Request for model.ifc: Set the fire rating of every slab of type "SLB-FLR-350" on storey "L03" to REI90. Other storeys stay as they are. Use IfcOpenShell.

First a look at what the model holds.

```python
import ifcopenshell
import ifcopenshell.util.element

model = ifcopenshell.open("model.ifc")
print(model.schema)
storey = next(s for s in model.by_type("IfcBuildingStorey") if s.Name == "L03")
slabs = [e for e in ifcopenshell.util.element.get_decomposition(storey) if e.is_a("IfcSlab")]
seen = {}
for e in slabs:
    element_type = ifcopenshell.util.element.get_type(e)
    key = (element_type.Name if element_type != e and element_type else None, ifcopenshell.util.element.get_pset(e, "Pset_SlabCommon", "FireRating"))
    seen[key] = seen.get(key, 0) + 1
for (name, value), count in sorted(seen.items(), key=str):
    print(count, "x", name, "|", value)
```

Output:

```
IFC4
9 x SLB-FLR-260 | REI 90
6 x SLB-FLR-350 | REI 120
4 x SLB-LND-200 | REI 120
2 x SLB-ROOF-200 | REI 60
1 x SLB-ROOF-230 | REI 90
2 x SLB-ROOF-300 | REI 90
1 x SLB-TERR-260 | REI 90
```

```python
import ifcopenshell
import ifcopenshell.api.pset
import ifcopenshell.util.element

model = ifcopenshell.open("model.ifc")

storey = next(s for s in model.by_type("IfcBuildingStorey") if s.Name == "L03")
slabs = [e for e in ifcopenshell.util.element.get_decomposition(storey) if e.is_a("IfcSlab")]

count = 0
for e in slabs:
    element_type = ifcopenshell.util.element.get_type(e)
    if element_type in (None, e) or element_type.Name != "SLB-FLR-350":
        continue
    # add_pset returns the element's existing set when there is one.
    pset = ifcopenshell.api.pset.add_pset(model, product=e, name="Pset_SlabCommon")
    ifcopenshell.api.pset.edit_pset(model, pset=pset, properties={"FireRating": "REI90"})
    count += 1

print(count, "slabs updated")

model.write("model_v2.ifc")
```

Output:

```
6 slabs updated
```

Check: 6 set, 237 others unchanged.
